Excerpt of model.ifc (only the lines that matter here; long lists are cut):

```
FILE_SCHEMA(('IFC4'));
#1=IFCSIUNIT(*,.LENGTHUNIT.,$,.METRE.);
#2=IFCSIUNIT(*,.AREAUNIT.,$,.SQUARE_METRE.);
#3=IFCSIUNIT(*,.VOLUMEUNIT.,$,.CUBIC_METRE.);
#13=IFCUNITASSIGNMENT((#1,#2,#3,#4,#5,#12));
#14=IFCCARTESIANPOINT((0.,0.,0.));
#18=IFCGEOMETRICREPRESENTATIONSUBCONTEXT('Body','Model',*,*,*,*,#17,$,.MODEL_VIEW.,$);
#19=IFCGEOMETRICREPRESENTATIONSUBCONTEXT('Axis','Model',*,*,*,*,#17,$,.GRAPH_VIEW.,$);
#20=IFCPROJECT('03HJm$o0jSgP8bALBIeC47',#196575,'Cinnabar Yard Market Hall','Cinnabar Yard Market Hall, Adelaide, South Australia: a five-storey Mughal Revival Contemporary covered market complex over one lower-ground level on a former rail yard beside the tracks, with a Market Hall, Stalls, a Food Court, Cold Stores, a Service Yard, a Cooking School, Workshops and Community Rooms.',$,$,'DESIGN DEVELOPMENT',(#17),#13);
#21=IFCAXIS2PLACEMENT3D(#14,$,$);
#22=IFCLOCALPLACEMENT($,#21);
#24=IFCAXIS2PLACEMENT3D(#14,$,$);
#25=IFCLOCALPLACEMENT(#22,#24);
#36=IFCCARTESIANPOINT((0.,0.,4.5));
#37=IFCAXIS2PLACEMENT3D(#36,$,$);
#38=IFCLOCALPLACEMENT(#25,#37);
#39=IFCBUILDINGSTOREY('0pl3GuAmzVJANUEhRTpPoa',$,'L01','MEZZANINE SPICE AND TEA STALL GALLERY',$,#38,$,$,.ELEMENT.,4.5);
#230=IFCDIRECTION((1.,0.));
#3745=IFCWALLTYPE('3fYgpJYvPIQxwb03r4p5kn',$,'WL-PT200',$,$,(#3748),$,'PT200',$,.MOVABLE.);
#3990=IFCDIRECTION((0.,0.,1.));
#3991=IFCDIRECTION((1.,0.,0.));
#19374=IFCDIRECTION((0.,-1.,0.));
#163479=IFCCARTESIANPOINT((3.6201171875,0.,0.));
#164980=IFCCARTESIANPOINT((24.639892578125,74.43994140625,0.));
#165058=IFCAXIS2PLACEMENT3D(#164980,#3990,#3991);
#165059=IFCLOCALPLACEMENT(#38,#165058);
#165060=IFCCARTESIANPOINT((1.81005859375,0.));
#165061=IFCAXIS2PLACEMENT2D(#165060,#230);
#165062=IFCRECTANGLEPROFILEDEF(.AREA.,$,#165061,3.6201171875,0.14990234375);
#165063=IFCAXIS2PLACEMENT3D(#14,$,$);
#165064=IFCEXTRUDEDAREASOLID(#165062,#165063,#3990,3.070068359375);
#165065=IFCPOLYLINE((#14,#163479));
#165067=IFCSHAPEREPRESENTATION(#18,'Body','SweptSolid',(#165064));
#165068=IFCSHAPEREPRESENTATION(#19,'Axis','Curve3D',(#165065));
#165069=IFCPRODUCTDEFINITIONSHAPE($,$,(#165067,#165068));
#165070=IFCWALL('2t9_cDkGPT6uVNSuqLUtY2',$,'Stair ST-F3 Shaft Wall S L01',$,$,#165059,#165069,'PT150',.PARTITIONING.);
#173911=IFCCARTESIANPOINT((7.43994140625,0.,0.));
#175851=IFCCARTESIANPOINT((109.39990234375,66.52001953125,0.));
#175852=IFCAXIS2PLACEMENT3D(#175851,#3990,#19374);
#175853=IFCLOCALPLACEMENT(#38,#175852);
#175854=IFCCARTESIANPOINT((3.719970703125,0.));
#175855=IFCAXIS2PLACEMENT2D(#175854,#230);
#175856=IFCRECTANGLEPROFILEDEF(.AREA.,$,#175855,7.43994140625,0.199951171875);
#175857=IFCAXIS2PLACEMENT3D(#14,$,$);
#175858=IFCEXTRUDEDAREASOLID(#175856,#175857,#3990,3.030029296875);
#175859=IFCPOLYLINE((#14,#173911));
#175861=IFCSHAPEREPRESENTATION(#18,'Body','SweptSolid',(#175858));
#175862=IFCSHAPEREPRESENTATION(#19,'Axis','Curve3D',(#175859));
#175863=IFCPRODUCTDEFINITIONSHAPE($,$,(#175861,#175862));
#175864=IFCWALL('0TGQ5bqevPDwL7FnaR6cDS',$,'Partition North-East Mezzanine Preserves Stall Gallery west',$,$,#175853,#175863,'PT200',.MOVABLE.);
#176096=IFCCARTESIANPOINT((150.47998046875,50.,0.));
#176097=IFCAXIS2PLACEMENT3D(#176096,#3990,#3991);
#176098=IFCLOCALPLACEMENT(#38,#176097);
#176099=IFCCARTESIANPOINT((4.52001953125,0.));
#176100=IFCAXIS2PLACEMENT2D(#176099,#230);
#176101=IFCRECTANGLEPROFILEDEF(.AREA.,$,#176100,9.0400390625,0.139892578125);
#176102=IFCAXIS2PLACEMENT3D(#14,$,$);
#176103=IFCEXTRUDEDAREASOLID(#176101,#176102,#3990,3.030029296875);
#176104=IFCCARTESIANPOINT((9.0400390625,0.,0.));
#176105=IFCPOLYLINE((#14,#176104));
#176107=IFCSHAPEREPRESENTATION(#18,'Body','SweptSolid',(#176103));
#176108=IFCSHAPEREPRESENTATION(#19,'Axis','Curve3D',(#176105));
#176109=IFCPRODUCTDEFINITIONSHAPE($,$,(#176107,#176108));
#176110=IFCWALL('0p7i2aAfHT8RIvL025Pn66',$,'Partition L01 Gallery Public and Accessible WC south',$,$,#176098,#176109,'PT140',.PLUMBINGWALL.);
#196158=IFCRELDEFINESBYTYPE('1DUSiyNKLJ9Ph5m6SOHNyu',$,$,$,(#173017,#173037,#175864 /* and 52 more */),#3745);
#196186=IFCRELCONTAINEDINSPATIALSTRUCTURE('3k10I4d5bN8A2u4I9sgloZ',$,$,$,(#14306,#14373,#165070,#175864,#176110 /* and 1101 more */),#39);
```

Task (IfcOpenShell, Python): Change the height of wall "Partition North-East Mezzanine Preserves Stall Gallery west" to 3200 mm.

```python
import ifcopenshell
import ifcopenshell.geom
import ifcopenshell.util.representation
import ifcopenshell.util.shape
import ifcopenshell.util.unit

model = ifcopenshell.open("model.ifc")
unit_scale = ifcopenshell.util.unit.calculate_unit_scale(model)
settings = ifcopenshell.geom.settings()


def volume(element):
    """Net volume in cubic metres, openings subtracted."""
    shape = ifcopenshell.geom.create_shape(settings, element)
    return ifcopenshell.util.shape.get_volume(shape.geometry)


wall = model.by_guid("0TGQ5bqevPDwL7FnaR6cDS")
before = volume(wall)

body = ifcopenshell.util.representation.get_representation(wall, "Model", "Body")
solid = body.Items[0]
old_height = solid.Depth
solid.Depth = 3.2 / unit_scale
after = volume(wall)

print(f"height {old_height:g} -> {solid.Depth:g}, volume {before:.3f} -> {after:.3f} m3")

model.write("model_edited.ifc")
```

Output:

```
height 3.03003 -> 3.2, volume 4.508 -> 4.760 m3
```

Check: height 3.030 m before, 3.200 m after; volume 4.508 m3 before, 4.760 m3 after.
